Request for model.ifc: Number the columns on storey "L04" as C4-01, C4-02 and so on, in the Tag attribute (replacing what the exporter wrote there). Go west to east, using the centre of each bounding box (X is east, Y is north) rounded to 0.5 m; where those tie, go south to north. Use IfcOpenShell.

First a look at what the model holds.

```python
import ifcopenshell
import ifcopenshell.util.element
import ifcopenshell.util.placement

model = ifcopenshell.open("model.ifc")
print(model.schema)
storey = next(s for s in model.by_type("IfcBuildingStorey") if s.Name == "L04")
columns = [e for e in ifcopenshell.util.element.get_decomposition(storey) if e.is_a("IfcColumn")]
for e in sorted(columns, key=lambda e: e.id()):
    origin = ifcopenshell.util.placement.get_local_placement(e.ObjectPlacement)[:3, 3]
    print(e.id(), e.Tag, e.Name, origin.round(2) + 0.0, sep=" | ")
```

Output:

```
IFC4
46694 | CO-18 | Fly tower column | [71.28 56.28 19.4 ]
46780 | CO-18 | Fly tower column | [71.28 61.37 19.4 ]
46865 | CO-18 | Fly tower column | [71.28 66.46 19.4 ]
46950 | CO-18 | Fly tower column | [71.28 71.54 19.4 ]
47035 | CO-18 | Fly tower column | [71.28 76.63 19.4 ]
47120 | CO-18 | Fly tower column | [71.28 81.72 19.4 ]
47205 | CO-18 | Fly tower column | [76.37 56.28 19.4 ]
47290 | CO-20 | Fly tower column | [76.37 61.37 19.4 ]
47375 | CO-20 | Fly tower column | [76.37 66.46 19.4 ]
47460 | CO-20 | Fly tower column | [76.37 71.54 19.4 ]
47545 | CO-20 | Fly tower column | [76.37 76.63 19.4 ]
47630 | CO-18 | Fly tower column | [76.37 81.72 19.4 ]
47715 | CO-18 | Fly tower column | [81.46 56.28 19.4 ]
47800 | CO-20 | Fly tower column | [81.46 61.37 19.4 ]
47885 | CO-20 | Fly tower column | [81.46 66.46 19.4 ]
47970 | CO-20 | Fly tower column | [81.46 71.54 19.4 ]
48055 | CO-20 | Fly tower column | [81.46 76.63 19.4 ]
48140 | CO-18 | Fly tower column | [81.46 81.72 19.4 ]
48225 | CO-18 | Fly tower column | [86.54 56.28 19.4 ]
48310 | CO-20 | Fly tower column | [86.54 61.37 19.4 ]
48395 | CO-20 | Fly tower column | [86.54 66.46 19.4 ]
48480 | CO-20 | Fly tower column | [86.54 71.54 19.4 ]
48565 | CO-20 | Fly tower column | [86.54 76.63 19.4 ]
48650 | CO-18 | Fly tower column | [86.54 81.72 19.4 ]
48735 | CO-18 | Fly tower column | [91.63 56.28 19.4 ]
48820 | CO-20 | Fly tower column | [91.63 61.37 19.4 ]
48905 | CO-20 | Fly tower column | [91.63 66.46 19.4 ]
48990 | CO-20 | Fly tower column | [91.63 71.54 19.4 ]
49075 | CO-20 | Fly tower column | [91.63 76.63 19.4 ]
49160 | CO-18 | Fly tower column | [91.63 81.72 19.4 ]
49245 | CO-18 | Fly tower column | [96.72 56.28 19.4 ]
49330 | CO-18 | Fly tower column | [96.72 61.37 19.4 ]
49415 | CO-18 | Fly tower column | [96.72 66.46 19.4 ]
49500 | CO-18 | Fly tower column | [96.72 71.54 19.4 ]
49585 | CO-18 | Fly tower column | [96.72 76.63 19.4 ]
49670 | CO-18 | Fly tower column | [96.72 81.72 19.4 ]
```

```python
import ifcopenshell
import ifcopenshell.geom
import ifcopenshell.util.element
import ifcopenshell.util.shape

model = ifcopenshell.open("model.ifc")
settings = ifcopenshell.geom.settings()
settings.set("use-world-coords", True)


def centre(element):
    shape = ifcopenshell.geom.create_shape(settings, element)
    return ifcopenshell.util.shape.get_bbox_centroid(shape.geometry)


storey = next(s for s in model.by_type("IfcBuildingStorey") if s.Name == "L04")
columns = [e for e in ifcopenshell.util.element.get_decomposition(storey) if e.is_a("IfcColumn")]

# Insertion points can sit at a corner or the storey origin, so sort by the geometry (in metres).
centres = {e: centre(e) for e in columns}
columns.sort(key=lambda e: (round(centres[e][0] / 0.5), centres[e][1]))

for i, e in enumerate(columns, start=1):
    number = f"C4-{i:02d}"
    e.Tag = number
    print(e.id(), number)

model.write("model_updated.ifc")
```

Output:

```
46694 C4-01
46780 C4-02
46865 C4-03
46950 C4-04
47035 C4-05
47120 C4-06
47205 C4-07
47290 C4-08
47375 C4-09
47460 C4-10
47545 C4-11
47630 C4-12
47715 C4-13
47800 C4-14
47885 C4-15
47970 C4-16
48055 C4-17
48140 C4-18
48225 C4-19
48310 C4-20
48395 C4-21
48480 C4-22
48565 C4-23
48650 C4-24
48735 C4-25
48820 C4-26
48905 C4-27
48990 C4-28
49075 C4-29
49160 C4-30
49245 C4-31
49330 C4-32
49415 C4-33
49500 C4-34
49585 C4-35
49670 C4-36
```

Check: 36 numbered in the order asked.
